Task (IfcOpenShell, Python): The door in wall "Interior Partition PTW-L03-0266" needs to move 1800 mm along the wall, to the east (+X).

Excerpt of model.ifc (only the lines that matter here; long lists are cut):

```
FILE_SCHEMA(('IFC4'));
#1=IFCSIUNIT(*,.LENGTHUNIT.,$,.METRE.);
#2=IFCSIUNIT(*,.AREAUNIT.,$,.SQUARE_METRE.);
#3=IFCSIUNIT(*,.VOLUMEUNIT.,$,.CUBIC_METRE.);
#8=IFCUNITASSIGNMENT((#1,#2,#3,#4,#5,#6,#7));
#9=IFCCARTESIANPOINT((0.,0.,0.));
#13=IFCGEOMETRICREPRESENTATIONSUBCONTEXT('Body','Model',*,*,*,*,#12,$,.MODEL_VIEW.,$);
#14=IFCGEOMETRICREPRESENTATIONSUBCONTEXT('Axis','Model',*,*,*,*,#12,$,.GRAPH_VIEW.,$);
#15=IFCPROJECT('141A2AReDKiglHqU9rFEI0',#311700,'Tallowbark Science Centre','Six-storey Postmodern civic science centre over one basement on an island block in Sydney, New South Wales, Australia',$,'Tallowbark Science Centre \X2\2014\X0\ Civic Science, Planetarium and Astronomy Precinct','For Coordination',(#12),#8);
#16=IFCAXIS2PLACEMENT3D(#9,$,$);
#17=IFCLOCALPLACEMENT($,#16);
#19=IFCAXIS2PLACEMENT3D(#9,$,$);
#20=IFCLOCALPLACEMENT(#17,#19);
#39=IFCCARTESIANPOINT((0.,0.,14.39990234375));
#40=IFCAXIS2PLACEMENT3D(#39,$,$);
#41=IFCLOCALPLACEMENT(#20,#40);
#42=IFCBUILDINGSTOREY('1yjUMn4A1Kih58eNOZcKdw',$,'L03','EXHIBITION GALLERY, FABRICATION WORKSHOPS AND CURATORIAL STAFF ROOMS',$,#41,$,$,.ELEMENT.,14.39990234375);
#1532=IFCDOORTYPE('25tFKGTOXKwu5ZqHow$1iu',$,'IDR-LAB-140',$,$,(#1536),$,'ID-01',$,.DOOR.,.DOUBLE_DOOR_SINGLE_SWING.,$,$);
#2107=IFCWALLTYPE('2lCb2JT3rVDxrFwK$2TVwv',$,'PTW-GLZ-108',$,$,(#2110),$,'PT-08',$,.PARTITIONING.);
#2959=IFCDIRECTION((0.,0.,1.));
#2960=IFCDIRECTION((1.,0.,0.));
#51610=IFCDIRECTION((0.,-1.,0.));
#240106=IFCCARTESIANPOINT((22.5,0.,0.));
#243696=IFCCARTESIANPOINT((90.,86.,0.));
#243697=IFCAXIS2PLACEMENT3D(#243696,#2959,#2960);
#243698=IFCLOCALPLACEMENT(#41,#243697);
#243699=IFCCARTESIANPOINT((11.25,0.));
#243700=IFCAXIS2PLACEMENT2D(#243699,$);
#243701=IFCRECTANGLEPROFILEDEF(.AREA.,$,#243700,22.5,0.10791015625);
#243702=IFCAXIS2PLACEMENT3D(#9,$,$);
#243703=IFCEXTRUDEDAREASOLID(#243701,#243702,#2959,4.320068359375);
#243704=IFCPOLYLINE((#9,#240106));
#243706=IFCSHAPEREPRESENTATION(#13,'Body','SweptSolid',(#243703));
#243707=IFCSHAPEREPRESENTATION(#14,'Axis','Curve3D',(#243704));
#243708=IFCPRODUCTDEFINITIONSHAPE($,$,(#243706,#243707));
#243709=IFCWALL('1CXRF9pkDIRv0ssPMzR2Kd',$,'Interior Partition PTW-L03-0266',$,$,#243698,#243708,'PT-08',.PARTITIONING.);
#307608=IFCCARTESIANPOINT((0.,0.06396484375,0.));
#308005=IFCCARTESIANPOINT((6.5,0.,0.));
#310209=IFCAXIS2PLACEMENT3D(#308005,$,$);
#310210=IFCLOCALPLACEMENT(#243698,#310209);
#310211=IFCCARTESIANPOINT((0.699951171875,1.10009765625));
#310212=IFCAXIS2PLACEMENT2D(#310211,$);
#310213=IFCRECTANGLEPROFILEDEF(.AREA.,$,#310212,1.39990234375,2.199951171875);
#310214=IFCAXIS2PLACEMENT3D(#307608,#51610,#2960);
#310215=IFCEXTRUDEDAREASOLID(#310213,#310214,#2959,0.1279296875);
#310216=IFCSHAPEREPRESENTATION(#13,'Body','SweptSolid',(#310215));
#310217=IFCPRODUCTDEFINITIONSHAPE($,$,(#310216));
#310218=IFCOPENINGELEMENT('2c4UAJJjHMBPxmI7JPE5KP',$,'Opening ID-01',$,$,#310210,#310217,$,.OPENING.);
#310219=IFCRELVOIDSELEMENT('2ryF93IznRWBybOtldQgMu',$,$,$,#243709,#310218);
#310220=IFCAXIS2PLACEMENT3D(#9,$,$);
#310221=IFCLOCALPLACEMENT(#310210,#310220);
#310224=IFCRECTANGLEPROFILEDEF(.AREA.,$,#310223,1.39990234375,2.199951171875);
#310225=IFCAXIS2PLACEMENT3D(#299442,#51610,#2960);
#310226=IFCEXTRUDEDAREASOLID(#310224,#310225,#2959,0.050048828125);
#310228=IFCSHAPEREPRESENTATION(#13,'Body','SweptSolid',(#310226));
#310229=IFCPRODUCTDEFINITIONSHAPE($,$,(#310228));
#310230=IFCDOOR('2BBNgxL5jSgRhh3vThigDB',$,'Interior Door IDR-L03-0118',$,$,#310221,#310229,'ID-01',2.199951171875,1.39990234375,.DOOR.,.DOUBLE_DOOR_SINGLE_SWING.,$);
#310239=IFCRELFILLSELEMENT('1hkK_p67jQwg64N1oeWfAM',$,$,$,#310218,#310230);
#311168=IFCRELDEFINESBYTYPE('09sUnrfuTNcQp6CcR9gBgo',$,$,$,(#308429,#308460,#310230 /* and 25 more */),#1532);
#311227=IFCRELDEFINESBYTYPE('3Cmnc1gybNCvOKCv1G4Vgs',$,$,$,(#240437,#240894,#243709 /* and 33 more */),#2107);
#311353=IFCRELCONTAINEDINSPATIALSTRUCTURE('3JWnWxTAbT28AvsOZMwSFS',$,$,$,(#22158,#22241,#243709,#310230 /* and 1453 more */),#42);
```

```python
import ifcopenshell
import ifcopenshell.api.geometry
import ifcopenshell.util.placement

model = ifcopenshell.open("model.ifc")

door = model.by_id(310230)
opening = door.FillsVoids[0].RelatingOpeningElement
wall = opening.VoidsElements[0].RelatingBuildingElement

wall_matrix = ifcopenshell.util.placement.get_local_placement(wall.ObjectPlacement)
shift = wall_matrix[:3, 0] * 1.8
before = ifcopenshell.util.placement.get_local_placement(door.ObjectPlacement)[:3, 3].copy()

# The door is placed relative to its opening, so it follows when the opening moves.
matrix = ifcopenshell.util.placement.get_local_placement(opening.ObjectPlacement)
matrix[:3, 3] += shift
ifcopenshell.api.geometry.edit_object_placement(
    model, product=opening, matrix=matrix, is_si=False, should_transform_children=True
)

after = ifcopenshell.util.placement.get_local_placement(door.ObjectPlacement)[:3, 3]
print("door moved by", (after - before).round(3) + 0.0)

model.write("model-out.ifc")
```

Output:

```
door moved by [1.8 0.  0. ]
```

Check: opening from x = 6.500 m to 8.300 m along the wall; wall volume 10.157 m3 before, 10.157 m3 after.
